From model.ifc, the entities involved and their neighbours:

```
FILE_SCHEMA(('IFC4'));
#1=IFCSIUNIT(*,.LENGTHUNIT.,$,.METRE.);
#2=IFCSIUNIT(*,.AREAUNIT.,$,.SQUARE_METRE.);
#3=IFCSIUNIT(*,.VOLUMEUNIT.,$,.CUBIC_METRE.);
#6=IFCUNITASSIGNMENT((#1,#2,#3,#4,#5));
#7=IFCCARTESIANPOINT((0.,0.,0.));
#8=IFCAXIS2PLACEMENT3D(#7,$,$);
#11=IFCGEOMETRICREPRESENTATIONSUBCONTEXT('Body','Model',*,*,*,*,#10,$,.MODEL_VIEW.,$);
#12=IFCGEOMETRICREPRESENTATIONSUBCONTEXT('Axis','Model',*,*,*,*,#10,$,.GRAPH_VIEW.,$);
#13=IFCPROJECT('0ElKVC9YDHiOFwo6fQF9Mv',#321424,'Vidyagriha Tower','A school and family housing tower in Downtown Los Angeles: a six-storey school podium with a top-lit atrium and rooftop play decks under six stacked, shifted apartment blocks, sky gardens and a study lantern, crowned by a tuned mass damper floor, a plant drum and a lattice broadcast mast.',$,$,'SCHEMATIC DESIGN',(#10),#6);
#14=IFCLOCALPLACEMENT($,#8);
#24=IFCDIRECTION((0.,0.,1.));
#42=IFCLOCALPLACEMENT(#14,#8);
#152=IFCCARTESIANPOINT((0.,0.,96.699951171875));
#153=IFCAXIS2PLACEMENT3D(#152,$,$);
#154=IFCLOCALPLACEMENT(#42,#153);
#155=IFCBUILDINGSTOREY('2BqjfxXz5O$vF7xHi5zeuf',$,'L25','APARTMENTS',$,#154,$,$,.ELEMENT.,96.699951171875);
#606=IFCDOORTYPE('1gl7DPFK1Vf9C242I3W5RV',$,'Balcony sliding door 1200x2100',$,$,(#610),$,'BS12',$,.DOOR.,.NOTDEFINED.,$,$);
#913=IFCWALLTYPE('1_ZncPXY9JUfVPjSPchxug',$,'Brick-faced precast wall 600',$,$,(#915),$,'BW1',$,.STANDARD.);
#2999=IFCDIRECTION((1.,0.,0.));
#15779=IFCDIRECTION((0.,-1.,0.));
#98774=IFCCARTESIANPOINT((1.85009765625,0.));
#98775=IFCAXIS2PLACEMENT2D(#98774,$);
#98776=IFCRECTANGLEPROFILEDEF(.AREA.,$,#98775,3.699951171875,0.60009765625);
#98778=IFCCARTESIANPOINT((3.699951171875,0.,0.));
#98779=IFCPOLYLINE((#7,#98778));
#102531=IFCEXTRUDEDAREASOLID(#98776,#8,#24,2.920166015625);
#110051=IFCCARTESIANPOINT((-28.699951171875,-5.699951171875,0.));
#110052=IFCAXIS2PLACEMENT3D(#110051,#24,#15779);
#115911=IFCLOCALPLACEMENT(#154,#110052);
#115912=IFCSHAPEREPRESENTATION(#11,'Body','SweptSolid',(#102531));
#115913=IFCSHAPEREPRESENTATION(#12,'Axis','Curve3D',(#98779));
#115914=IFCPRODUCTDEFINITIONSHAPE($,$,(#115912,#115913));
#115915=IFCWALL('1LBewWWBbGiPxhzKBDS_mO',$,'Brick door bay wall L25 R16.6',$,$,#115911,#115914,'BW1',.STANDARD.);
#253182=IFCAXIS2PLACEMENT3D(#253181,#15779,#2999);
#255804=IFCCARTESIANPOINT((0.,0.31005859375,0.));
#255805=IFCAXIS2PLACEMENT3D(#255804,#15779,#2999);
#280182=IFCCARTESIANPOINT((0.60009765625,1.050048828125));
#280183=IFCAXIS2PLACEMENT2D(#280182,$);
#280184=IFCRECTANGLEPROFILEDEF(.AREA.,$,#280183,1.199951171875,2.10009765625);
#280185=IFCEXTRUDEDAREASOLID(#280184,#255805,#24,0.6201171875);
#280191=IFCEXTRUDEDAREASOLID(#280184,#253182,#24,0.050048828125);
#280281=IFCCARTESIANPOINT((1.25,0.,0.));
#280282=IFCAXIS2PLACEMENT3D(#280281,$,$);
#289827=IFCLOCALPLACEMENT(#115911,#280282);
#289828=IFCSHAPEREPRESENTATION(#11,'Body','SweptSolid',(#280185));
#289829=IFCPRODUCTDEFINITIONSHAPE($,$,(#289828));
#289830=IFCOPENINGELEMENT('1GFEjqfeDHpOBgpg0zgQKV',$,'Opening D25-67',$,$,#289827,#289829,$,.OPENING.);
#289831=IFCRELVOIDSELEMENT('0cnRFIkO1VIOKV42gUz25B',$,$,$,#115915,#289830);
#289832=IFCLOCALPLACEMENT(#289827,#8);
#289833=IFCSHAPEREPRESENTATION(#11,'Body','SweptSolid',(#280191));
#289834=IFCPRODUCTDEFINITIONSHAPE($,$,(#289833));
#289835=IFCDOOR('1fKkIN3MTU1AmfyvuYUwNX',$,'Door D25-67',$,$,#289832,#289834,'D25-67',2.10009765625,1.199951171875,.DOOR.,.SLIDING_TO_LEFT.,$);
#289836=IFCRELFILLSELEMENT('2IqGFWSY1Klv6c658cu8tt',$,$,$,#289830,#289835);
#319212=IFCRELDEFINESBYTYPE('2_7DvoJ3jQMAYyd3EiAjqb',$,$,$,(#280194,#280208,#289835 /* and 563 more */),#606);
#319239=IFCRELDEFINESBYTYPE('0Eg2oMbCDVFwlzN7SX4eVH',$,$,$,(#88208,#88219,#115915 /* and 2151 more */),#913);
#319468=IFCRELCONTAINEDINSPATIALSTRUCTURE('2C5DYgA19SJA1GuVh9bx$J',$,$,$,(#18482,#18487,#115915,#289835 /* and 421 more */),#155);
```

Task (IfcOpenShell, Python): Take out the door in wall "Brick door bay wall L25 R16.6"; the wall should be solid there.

```python
import ifcopenshell
import ifcopenshell.api.feature
import ifcopenshell.api.root
import ifcopenshell.geom
import ifcopenshell.util.shape

model = ifcopenshell.open("model.ifc")
settings = ifcopenshell.geom.settings()


def volume(element):
    """Net volume in cubic metres, openings subtracted."""
    shape = ifcopenshell.geom.create_shape(settings, element)
    return ifcopenshell.util.shape.get_volume(shape.geometry)


door = model.by_guid("1fKkIN3MTU1AmfyvuYUwNX")
opening = door.FillsVoids[0].RelatingOpeningElement
wall = opening.VoidsElements[0].RelatingBuildingElement
before = volume(wall)

ifcopenshell.api.root.remove_product(model, product=door)
ifcopenshell.api.feature.remove_feature(model, feature=opening)

after = volume(wall)

print(f"wall volume {before:.3f} -> {after:.3f} m3")

model.write("model_edited.ifc")
```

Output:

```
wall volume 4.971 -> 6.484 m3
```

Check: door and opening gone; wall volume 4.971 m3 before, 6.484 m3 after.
